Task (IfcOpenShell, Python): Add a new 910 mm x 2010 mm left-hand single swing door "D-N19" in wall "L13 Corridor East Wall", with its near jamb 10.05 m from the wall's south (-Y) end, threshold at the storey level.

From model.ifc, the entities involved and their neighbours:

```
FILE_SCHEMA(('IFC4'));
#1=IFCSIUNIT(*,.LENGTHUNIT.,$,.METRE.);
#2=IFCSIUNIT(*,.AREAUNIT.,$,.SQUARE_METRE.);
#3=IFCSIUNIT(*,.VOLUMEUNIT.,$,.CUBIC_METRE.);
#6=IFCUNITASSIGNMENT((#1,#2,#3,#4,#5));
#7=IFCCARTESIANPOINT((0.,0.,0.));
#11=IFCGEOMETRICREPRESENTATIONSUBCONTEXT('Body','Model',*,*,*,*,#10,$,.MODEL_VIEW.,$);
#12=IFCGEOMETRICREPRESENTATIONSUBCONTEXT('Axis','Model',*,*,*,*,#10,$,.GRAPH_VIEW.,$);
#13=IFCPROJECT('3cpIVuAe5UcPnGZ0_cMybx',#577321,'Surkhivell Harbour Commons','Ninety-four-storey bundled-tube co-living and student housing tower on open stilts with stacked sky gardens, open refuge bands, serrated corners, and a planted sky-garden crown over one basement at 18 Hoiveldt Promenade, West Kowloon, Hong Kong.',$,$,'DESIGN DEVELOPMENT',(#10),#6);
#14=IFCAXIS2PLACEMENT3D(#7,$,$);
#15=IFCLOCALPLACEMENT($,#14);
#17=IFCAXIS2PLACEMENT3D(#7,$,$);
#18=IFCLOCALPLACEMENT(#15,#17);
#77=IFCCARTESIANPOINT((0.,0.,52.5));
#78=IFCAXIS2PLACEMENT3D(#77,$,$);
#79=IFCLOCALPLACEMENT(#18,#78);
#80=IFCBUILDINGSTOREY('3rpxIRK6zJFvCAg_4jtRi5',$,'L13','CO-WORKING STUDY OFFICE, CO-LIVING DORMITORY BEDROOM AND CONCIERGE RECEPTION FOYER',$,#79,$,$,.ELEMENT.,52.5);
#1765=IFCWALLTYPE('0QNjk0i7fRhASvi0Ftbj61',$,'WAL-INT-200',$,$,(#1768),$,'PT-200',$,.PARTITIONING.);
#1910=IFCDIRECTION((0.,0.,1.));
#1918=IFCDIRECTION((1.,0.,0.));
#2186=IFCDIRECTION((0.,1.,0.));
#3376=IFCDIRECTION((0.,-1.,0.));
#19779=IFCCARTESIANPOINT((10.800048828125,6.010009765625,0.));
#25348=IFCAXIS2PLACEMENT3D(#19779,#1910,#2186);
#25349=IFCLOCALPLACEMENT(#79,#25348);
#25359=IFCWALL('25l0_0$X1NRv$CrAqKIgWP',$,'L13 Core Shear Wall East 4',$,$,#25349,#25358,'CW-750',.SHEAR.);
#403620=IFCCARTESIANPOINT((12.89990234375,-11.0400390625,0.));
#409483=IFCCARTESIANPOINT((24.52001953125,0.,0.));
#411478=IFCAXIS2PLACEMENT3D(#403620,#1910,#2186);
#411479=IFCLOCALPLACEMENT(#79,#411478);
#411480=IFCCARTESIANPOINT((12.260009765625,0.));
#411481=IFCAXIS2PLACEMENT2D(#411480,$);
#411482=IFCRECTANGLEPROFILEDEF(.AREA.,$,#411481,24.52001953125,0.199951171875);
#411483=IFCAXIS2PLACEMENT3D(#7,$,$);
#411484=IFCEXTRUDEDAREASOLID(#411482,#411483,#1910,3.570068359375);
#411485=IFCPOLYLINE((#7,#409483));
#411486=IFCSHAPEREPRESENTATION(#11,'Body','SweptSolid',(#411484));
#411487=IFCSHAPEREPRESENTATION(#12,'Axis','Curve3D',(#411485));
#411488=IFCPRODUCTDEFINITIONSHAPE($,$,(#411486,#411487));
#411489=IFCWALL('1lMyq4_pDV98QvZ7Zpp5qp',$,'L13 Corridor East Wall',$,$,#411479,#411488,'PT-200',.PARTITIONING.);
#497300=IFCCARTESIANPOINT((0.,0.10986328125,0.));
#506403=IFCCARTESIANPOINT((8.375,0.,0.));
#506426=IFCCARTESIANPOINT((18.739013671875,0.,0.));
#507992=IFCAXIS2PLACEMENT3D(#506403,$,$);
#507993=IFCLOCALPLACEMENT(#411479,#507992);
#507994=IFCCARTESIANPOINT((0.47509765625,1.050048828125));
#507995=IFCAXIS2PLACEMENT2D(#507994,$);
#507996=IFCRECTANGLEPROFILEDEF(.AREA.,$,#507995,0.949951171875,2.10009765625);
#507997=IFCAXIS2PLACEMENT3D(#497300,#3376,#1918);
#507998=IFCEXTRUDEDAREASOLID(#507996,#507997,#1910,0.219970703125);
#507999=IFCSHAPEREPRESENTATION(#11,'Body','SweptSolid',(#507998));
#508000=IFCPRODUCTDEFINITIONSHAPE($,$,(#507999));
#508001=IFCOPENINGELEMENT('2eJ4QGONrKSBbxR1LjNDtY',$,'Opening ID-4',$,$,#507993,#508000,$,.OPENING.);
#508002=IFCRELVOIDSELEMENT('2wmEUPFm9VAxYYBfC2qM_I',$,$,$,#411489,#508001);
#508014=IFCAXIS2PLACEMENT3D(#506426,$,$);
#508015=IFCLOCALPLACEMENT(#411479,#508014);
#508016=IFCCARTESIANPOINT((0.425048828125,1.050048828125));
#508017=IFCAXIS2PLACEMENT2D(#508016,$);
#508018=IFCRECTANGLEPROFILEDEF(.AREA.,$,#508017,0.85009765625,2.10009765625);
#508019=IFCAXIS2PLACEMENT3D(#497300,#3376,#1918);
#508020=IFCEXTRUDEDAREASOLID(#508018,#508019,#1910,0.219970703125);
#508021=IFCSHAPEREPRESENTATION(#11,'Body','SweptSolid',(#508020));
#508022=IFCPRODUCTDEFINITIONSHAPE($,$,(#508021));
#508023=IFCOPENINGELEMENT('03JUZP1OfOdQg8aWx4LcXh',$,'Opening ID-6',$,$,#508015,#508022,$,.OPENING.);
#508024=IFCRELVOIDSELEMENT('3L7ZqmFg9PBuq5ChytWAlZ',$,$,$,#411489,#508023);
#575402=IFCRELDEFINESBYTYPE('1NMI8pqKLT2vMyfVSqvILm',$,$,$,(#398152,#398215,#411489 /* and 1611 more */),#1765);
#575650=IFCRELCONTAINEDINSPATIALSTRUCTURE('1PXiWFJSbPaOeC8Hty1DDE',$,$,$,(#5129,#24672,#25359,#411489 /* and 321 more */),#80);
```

```python
import numpy as np
import ifcopenshell
import ifcopenshell.api.feature
import ifcopenshell.api.geometry
import ifcopenshell.api.root
import ifcopenshell.api.spatial
import ifcopenshell.geom
import ifcopenshell.util.element
import ifcopenshell.util.placement
import ifcopenshell.util.representation
import ifcopenshell.util.shape
import ifcopenshell.util.unit

model = ifcopenshell.open("model.ifc")
unit_scale = ifcopenshell.util.unit.calculate_unit_scale(model)
settings = ifcopenshell.geom.settings()


def volume(element):
    """Net volume in cubic metres, openings subtracted."""
    shape = ifcopenshell.geom.create_shape(settings, element)
    return ifcopenshell.util.shape.get_volume(shape.geometry)


wall = model.by_id(411489)
storey = ifcopenshell.util.element.get_container(wall, ifc_class="IfcBuildingStorey")
context = ifcopenshell.util.representation.get_context(model, "Model", "Body", "MODEL_VIEW")
before = volume(wall)

width, height, from_end, sill = 0.91, 2.01, 10.05, 0.0  # metres

# The wall runs along its own X axis, and the end named is its -X end.
wall_shape = ifcopenshell.geom.create_shape(settings, wall)
x, y, z = ifcopenshell.util.shape.get_vertices(wall_shape.geometry).T
start = x.min() + from_end
face, thickness = float(y.min()), float(y.max() - y.min())
wall_matrix = ifcopenshell.util.placement.get_local_placement(wall.ObjectPlacement)
level = ifcopenshell.util.placement.get_local_placement(storey.ObjectPlacement)[2, 3]


def in_wall(x, y):
    """Placement at x, y metres in the wall's axes, at sill height."""
    matrix = wall_matrix.copy()
    matrix[:, 3] = wall_matrix @ np.array([x / unit_scale, y / unit_scale, 0.0, 1.0])
    matrix[2, 3] = level + sill / unit_scale
    return matrix


# Opening: a box that overshoots both wall faces by 50 mm.
opening = ifcopenshell.api.root.create_entity(model, ifc_class="IfcOpeningElement", predefined_type="OPENING")
box = ifcopenshell.api.geometry.add_wall_representation(
    model, context=context, length=width, height=height, thickness=thickness + 0.1
)
ifcopenshell.api.geometry.assign_representation(model, product=opening, representation=box)
ifcopenshell.api.geometry.edit_object_placement(model, product=opening, matrix=in_wall(start, face - 0.05), is_si=False)
ifcopenshell.api.feature.add_feature(model, feature=opening, element=wall)

door = ifcopenshell.api.root.create_entity(model, ifc_class="IfcDoor", name="D-N19", predefined_type="DOOR")
door.OverallWidth, door.OverallHeight = width / unit_scale, height / unit_scale
door.OperationType = "SINGLE_SWING_LEFT"
body = ifcopenshell.api.geometry.add_door_representation(
    model,
    context=context,
    overall_width=door.OverallWidth,
    overall_height=door.OverallHeight,
    operation_type="SINGLE_SWING_LEFT",
    lining_properties={"LiningDepth": thickness / unit_scale, "ThresholdDepth": thickness / unit_scale},
)
ifcopenshell.api.geometry.assign_representation(model, product=door, representation=body)
ifcopenshell.api.spatial.assign_container(model, products=[door], relating_structure=storey)
ifcopenshell.api.feature.add_filling(model, opening=opening, element=door)

# The lining spans the wall, so the door starts at the wall face.
ifcopenshell.api.geometry.edit_object_placement(model, product=door, matrix=in_wall(start, face), is_si=False)

after = volume(wall)

print(f"wall volume {before:.3f} -> {after:.3f} m3")

model.write("model_updated.ifc")
```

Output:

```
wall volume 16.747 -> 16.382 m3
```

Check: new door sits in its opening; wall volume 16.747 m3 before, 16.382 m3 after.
